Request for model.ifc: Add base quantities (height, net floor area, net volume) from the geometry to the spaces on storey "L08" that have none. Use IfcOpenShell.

First a look at what the model holds.

```python
import ifcopenshell
import ifcopenshell.util.element
import ifcopenshell.util.unit

model = ifcopenshell.open("model.ifc")
print(model.schema)
for unit_type in ("LENGTHUNIT", "AREAUNIT", "VOLUMEUNIT"):
    print(unit_type, ifcopenshell.util.unit.calculate_unit_scale(model, unit_type))
storey = next(s for s in model.by_type("IfcBuildingStorey") if s.Name == "L08")
spaces = [e for e in ifcopenshell.util.element.get_decomposition(storey) if e.is_a("IfcSpace")]
for e in sorted(spaces, key=lambda e: e.id()):
    print(e.id(), e.is_a(), e.Name, list(ifcopenshell.util.element.get_psets(e, qtos_only=True)), sep=" | ")
```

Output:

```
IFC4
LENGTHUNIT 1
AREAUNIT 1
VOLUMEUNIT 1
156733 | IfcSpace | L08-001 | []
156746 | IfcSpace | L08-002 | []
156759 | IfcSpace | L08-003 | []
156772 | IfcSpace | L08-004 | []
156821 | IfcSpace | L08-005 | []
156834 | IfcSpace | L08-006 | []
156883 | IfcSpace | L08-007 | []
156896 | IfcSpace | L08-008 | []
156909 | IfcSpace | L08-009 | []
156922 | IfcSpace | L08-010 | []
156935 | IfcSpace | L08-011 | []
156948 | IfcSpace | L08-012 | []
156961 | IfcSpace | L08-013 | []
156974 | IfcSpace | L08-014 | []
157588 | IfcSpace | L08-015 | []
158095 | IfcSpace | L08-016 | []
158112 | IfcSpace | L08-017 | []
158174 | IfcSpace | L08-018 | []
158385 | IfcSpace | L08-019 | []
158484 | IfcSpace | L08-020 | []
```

```python
import ifcopenshell
import ifcopenshell.api.pset
import ifcopenshell.geom
import ifcopenshell.util.element
import ifcopenshell.util.shape
import ifcopenshell.util.unit

model = ifcopenshell.open("model.ifc")
unit_scale = ifcopenshell.util.unit.calculate_unit_scale(model)
area_scale = ifcopenshell.util.unit.calculate_unit_scale(model, "AREAUNIT")
volume_scale = ifcopenshell.util.unit.calculate_unit_scale(model, "VOLUMEUNIT")
settings = ifcopenshell.geom.settings()

storey = next(s for s in model.by_type("IfcBuildingStorey") if s.Name == "L08")
spaces = [e for e in ifcopenshell.util.element.get_decomposition(storey) if e.is_a("IfcSpace")]

for e in sorted(spaces, key=lambda e: e.id()):
    if ifcopenshell.util.element.get_psets(e, qtos_only=True, should_inherit=False):
        continue
    # Geometry comes back in metres, in the element's own axes.
    shape = ifcopenshell.geom.create_shape(settings, e)
    values = {
        "Height": ifcopenshell.util.shape.get_z(shape.geometry) / unit_scale,
        "NetFloorArea": ifcopenshell.util.shape.get_footprint_area(shape.geometry) / area_scale,
        "NetVolume": ifcopenshell.util.shape.get_volume(shape.geometry) / volume_scale,
    }
    qto = ifcopenshell.api.pset.add_qto(model, product=e, name="Qto_SpaceBaseQuantities")
    ifcopenshell.api.pset.edit_qto(model, qto=qto, properties=values)
    print(e.id(), {k: round(v, 3) for k, v in values.items()})

model.write("model_rev.ifc")
```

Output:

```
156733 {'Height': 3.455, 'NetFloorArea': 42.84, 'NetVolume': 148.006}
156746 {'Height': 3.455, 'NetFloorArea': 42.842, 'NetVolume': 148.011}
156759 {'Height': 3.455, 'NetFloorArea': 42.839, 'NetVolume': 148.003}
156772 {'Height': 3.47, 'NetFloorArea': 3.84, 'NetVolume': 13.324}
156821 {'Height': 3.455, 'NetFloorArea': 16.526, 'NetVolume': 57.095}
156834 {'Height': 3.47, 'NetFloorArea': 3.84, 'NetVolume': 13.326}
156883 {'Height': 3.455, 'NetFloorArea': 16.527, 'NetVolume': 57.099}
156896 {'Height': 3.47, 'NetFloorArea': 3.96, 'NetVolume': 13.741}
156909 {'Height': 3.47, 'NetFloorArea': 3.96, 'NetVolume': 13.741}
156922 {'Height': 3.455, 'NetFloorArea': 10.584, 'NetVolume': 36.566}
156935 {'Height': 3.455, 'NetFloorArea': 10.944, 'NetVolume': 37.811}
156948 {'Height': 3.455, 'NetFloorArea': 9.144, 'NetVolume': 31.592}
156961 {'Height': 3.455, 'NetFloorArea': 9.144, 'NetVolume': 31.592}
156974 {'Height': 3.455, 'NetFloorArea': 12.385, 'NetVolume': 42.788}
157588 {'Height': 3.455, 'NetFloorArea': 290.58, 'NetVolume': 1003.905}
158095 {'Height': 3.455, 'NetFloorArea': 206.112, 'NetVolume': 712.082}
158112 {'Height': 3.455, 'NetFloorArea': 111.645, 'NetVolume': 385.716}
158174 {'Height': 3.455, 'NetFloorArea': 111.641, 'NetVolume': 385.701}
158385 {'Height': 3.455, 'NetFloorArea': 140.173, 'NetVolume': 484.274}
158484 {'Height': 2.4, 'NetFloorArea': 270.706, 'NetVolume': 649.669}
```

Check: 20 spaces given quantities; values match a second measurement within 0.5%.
